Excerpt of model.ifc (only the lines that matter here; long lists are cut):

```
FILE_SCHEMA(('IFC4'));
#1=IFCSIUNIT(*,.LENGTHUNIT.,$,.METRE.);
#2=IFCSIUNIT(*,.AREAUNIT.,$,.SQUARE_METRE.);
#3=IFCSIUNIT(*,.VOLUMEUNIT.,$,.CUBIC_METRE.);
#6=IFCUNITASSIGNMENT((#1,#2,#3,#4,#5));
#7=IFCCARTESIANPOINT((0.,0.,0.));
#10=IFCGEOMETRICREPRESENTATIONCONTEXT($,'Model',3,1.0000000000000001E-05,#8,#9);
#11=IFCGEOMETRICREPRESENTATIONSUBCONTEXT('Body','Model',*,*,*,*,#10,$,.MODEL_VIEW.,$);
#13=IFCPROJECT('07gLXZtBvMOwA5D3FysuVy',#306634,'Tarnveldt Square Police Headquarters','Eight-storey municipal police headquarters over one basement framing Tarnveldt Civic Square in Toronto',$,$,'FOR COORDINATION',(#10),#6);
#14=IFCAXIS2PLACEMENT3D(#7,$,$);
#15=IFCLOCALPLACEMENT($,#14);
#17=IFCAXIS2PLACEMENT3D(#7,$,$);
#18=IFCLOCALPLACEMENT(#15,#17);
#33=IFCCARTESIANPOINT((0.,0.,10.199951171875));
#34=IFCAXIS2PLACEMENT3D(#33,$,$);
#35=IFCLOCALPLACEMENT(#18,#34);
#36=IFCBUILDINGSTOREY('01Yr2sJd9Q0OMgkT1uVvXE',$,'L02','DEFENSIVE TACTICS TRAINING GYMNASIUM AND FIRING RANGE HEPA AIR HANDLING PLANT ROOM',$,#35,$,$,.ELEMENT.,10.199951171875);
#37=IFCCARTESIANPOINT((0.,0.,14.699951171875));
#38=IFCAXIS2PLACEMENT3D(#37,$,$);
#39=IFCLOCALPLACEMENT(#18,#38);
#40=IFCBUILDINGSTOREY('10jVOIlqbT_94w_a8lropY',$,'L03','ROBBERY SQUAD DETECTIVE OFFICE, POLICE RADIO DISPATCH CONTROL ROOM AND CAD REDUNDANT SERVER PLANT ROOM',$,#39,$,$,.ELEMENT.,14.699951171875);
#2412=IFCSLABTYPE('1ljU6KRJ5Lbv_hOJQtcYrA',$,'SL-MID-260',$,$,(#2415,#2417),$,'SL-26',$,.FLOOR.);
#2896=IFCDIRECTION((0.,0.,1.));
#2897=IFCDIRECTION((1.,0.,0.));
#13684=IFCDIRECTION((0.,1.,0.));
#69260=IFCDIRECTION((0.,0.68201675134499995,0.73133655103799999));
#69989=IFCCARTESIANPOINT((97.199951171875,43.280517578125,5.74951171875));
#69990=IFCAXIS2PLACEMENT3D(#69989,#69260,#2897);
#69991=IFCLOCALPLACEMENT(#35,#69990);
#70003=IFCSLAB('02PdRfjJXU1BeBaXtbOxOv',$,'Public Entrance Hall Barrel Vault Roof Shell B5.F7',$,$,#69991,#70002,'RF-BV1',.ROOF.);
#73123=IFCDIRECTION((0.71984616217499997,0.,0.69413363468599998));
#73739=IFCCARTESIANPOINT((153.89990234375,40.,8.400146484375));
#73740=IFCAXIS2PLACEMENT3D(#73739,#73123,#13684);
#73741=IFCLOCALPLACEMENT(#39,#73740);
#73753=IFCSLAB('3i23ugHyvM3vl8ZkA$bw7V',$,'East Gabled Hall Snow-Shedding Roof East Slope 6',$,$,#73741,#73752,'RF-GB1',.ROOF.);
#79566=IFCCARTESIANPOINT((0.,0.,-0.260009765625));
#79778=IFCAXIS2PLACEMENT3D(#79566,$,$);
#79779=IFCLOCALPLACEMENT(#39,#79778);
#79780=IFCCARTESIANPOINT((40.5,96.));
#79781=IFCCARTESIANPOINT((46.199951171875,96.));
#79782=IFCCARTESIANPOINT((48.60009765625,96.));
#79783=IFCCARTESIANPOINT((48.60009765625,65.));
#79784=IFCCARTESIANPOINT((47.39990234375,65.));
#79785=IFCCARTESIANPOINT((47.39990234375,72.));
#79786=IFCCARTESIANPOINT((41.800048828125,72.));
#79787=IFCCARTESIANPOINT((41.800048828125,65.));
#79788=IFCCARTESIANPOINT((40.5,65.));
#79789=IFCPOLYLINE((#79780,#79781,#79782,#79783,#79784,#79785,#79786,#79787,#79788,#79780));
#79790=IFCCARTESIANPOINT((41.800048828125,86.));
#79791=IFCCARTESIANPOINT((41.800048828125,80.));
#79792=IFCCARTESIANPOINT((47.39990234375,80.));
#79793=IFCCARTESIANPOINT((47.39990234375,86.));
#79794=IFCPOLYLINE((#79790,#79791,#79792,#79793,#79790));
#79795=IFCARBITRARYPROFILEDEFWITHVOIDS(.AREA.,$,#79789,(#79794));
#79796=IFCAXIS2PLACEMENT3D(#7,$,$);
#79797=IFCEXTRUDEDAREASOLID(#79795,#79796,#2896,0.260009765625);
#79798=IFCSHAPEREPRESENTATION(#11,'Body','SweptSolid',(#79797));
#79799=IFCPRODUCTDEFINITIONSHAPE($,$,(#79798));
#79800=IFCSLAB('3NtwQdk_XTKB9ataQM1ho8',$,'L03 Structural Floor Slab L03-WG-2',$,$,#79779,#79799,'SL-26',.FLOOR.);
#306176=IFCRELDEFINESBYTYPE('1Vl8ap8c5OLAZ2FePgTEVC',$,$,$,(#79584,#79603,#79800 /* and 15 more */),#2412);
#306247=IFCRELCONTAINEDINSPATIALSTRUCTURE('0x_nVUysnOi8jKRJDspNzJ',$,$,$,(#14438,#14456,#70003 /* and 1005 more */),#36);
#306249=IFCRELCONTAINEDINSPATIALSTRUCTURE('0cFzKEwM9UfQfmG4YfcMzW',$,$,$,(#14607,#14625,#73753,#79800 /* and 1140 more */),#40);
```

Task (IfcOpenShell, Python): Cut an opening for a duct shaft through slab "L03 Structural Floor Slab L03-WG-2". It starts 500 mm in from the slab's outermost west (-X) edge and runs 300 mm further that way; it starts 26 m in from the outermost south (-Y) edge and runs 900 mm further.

```python
import numpy as np
import ifcopenshell
import ifcopenshell.api.feature
import ifcopenshell.api.geometry
import ifcopenshell.api.root
import ifcopenshell.geom
import ifcopenshell.util.placement
import ifcopenshell.util.representation
import ifcopenshell.util.shape
import ifcopenshell.util.unit

model = ifcopenshell.open("model.ifc")
unit_scale = ifcopenshell.util.unit.calculate_unit_scale(model)
settings = ifcopenshell.geom.settings()


def volume(element):
    """Net volume in cubic metres, openings subtracted."""
    shape = ifcopenshell.geom.create_shape(settings, element)
    return ifcopenshell.util.shape.get_volume(shape.geometry)


slab = model.by_guid("3NtwQdk_XTKB9ataQM1ho8")
before = volume(slab)

# Extent in the slab's own axes, in metres. The edges named are its -X and -Y sides.
slab_shape = ifcopenshell.geom.create_shape(settings, slab)
vertices = ifcopenshell.util.shape.get_vertices(slab_shape.geometry)
x_min, y_min, bottom = vertices.min(axis=0)
top = vertices[:, 2].max()

opening = ifcopenshell.api.root.create_entity(model, ifc_class="IfcOpeningElement", name="Duct shaft opening", predefined_type="OPENING")
context = ifcopenshell.util.representation.get_context(model, "Model", "Body", "MODEL_VIEW")
width, depth = 0.3, 0.9
outline = [(0.0, 0.0), (width, 0.0), (width, depth), (0.0, depth), (0.0, 0.0)]
# Overshoot both faces by 50 mm so the cut is clean.
shape = ifcopenshell.api.geometry.add_slab_representation(
    model, context=context, depth=top - bottom + 0.1, polyline=outline
)
ifcopenshell.api.geometry.assign_representation(model, product=opening, representation=shape)

matrix = ifcopenshell.util.placement.get_local_placement(slab.ObjectPlacement)
matrix[:, 3] = matrix @ np.append(np.array([x_min + 0.5, y_min + 26, bottom - 0.05]) / unit_scale, 1.0)
ifcopenshell.api.geometry.edit_object_placement(model, product=opening, matrix=matrix, is_si=False)
ifcopenshell.api.feature.add_feature(model, feature=opening, element=slab)

after = volume(slab)

print(f"slab volume {before:.3f} -> {after:.3f} m3")

model.write("model_updated.ifc")
```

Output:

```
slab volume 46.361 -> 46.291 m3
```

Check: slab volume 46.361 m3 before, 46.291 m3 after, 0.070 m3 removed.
